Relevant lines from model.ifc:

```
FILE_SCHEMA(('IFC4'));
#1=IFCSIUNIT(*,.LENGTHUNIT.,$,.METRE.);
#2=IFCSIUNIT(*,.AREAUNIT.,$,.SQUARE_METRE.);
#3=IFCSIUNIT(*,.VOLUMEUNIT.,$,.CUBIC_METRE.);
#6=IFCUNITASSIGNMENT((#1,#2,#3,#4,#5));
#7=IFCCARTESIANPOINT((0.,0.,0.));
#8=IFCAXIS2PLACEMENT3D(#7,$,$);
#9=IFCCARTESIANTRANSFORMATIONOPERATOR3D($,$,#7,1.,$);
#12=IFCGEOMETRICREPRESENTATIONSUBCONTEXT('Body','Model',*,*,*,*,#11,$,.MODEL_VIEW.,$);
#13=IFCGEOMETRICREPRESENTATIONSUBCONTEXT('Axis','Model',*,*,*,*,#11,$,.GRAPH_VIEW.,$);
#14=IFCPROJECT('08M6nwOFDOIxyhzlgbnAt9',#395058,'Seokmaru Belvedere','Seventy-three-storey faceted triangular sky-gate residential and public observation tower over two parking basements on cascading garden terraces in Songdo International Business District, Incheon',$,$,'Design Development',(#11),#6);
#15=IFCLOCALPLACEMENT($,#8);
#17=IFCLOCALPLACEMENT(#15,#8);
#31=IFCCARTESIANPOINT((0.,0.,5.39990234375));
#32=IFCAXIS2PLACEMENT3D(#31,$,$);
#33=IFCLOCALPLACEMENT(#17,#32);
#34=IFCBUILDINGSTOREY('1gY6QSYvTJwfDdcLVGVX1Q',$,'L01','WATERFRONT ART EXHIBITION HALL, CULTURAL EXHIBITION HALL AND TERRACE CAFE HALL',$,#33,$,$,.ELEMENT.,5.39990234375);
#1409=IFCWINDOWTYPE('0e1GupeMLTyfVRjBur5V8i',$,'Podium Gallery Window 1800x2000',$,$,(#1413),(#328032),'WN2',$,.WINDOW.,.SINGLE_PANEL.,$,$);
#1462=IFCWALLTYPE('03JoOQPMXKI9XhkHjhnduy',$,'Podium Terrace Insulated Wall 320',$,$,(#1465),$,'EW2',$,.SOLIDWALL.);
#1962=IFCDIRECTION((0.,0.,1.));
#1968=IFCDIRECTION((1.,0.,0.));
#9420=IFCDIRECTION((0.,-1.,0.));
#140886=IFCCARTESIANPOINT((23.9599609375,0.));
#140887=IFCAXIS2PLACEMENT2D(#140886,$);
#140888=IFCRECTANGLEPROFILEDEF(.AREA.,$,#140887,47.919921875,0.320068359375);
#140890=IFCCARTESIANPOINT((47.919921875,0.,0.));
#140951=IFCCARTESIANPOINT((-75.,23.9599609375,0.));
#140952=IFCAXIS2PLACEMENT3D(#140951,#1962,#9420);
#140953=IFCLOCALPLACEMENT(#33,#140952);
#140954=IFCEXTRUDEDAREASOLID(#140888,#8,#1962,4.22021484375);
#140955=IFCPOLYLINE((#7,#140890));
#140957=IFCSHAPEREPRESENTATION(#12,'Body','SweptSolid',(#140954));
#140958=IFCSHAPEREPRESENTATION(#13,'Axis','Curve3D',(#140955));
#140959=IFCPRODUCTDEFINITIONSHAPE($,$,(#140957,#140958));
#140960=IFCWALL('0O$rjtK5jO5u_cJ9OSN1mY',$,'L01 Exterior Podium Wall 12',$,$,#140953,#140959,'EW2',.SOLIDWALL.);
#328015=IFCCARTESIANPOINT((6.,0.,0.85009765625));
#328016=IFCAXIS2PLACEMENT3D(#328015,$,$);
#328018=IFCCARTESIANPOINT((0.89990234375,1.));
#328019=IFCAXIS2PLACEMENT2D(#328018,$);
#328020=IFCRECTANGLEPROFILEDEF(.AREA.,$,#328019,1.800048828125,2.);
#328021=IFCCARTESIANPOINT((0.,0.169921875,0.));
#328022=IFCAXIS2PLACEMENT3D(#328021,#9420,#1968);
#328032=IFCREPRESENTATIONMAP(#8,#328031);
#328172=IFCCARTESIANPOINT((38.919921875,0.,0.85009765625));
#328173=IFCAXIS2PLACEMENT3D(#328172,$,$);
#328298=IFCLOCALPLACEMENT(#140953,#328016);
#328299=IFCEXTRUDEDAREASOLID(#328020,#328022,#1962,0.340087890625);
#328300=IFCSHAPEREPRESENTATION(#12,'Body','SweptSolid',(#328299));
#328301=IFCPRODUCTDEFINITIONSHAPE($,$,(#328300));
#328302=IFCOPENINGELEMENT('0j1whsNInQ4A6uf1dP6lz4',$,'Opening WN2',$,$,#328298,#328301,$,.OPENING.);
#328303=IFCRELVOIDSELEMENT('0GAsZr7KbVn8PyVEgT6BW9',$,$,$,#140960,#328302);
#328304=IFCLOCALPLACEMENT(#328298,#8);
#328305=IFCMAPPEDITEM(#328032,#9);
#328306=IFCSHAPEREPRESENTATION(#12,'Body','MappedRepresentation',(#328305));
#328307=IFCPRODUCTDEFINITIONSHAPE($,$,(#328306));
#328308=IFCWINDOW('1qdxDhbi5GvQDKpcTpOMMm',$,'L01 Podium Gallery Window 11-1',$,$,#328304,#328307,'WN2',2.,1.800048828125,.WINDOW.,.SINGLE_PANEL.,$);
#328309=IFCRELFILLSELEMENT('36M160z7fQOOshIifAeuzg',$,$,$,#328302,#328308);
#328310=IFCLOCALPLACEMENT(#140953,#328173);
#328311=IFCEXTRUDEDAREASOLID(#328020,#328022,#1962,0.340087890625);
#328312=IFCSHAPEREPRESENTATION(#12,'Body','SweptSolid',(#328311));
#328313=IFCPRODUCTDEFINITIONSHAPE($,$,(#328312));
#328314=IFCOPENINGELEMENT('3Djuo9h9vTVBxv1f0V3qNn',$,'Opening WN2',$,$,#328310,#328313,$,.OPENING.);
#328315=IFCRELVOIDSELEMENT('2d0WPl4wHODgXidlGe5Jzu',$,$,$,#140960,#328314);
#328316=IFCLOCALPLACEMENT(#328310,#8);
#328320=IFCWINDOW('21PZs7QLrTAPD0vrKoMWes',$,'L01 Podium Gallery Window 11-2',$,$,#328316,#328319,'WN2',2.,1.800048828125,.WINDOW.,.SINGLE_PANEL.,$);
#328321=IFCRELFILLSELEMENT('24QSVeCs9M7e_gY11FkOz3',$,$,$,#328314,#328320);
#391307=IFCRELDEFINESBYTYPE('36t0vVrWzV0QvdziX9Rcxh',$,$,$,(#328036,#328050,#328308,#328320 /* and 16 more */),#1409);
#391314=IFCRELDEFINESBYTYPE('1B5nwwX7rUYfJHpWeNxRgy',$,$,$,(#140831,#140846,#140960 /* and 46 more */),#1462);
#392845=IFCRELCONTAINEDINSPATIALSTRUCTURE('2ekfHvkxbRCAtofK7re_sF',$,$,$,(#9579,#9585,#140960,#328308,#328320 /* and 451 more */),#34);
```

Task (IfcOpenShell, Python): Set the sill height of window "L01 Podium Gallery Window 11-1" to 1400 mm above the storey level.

```python
import numpy as np
import ifcopenshell
import ifcopenshell.api.geometry
import ifcopenshell.geom
import ifcopenshell.util.element
import ifcopenshell.util.placement
import ifcopenshell.util.shape
import ifcopenshell.util.unit

model = ifcopenshell.open("model.ifc")
unit_scale = ifcopenshell.util.unit.calculate_unit_scale(model)

window = model.by_guid("1qdxDhbi5GvQDKpcTpOMMm")
opening = window.FillsVoids[0].RelatingOpeningElement
storey = ifcopenshell.util.element.get_container(window, ifc_class="IfcBuildingStorey")
level = ifcopenshell.util.placement.get_local_placement(storey.ObjectPlacement)[2, 3]

# The opening's origin need not be at the sill, so measure its lowest point.
shape = ifcopenshell.geom.create_shape(ifcopenshell.geom.settings(), opening)
bottom = ifcopenshell.util.shape.get_shape_bottom_elevation(shape, shape.geometry) / unit_scale
dz = level + 1.4 / unit_scale - bottom

shift = np.array([0.0, 0.0, dz])
# The window is placed relative to its opening, so it follows when the opening moves.
matrix = ifcopenshell.util.placement.get_local_placement(opening.ObjectPlacement)
matrix[:3, 3] += shift
ifcopenshell.api.geometry.edit_object_placement(
    model, product=opening, matrix=matrix, is_si=False, should_transform_children=True
)

print(f"moved by {dz * unit_scale:+.3f} m")

model.write("model-out.ifc")
```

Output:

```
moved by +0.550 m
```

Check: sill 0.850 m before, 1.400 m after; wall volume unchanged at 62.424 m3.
